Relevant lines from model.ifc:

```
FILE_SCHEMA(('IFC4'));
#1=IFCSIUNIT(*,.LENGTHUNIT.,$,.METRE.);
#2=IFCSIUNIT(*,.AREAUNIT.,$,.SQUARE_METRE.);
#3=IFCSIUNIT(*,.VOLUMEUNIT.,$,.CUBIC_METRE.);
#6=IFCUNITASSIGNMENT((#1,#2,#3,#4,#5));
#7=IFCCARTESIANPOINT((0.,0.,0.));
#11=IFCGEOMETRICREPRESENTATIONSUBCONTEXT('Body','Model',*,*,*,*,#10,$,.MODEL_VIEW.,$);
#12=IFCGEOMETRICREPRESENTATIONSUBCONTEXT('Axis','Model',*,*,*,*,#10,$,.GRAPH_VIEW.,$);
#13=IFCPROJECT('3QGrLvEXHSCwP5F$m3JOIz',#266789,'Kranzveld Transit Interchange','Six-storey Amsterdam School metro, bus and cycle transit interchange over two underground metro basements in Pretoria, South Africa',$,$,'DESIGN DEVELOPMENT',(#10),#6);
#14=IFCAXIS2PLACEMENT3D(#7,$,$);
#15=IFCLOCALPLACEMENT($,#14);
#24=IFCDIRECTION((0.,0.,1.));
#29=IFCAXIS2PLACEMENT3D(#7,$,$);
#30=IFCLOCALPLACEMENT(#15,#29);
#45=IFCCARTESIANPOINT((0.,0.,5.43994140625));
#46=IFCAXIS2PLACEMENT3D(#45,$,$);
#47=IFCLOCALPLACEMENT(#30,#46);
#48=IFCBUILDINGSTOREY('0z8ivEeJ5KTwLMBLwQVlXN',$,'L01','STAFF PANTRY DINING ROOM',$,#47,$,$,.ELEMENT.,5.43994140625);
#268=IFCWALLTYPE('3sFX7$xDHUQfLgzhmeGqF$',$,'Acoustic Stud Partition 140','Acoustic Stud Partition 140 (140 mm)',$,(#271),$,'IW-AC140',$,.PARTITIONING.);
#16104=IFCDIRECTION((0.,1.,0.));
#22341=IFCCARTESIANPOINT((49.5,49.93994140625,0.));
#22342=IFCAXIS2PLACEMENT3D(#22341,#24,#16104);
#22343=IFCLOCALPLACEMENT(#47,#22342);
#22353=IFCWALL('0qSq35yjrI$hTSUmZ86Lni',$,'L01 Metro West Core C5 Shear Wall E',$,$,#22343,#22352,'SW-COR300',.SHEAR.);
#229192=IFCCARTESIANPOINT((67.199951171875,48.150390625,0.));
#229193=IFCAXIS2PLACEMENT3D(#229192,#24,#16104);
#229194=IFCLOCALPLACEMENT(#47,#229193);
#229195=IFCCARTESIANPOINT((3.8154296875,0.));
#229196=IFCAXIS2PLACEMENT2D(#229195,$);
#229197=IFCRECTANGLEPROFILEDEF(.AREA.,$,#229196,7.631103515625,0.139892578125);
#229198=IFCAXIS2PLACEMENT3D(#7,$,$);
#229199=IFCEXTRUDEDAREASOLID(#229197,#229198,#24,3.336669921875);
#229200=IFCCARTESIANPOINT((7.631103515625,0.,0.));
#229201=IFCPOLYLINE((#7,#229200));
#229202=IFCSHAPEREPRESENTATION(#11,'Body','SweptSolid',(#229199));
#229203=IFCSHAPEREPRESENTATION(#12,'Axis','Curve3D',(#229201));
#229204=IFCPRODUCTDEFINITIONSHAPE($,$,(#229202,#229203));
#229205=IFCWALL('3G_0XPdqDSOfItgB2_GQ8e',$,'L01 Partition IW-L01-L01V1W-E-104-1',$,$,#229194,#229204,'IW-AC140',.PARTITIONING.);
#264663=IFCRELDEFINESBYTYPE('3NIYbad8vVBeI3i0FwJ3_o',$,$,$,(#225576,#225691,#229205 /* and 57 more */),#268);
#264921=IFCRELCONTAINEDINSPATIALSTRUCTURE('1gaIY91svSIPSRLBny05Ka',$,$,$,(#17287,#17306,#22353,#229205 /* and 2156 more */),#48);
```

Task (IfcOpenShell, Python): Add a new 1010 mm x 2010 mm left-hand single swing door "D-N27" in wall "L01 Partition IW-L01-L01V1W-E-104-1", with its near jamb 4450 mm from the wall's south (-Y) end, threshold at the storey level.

```python
import numpy as np
import ifcopenshell
import ifcopenshell.api.feature
import ifcopenshell.api.geometry
import ifcopenshell.api.root
import ifcopenshell.api.spatial
import ifcopenshell.geom
import ifcopenshell.util.element
import ifcopenshell.util.placement
import ifcopenshell.util.representation
import ifcopenshell.util.shape
import ifcopenshell.util.unit

model = ifcopenshell.open("model.ifc")
unit_scale = ifcopenshell.util.unit.calculate_unit_scale(model)
settings = ifcopenshell.geom.settings()


def volume(element):
    """Net volume in cubic metres, openings subtracted."""
    shape = ifcopenshell.geom.create_shape(settings, element)
    return ifcopenshell.util.shape.get_volume(shape.geometry)


wall = model.by_guid("3G_0XPdqDSOfItgB2_GQ8e")
storey = ifcopenshell.util.element.get_container(wall, ifc_class="IfcBuildingStorey")
context = ifcopenshell.util.representation.get_context(model, "Model", "Body", "MODEL_VIEW")
before = volume(wall)

width, height, from_end, sill = 1.01, 2.01, 4.45, 0.0  # metres

# The wall runs along its own X axis, and the end named is its -X end.
wall_shape = ifcopenshell.geom.create_shape(settings, wall)
x, y, z = ifcopenshell.util.shape.get_vertices(wall_shape.geometry).T
start = x.min() + from_end
face, thickness = float(y.min()), float(y.max() - y.min())
wall_matrix = ifcopenshell.util.placement.get_local_placement(wall.ObjectPlacement)
level = ifcopenshell.util.placement.get_local_placement(storey.ObjectPlacement)[2, 3]


def in_wall(x, y):
    """Placement at x, y metres in the wall's axes, at sill height."""
    matrix = wall_matrix.copy()
    matrix[:, 3] = wall_matrix @ np.array([x / unit_scale, y / unit_scale, 0.0, 1.0])
    matrix[2, 3] = level + sill / unit_scale
    return matrix


# Opening: a box that overshoots both wall faces by 50 mm.
opening = ifcopenshell.api.root.create_entity(model, ifc_class="IfcOpeningElement", predefined_type="OPENING")
box = ifcopenshell.api.geometry.add_wall_representation(
    model, context=context, length=width, height=height, thickness=thickness + 0.1
)
ifcopenshell.api.geometry.assign_representation(model, product=opening, representation=box)
ifcopenshell.api.geometry.edit_object_placement(model, product=opening, matrix=in_wall(start, face - 0.05), is_si=False)
ifcopenshell.api.feature.add_feature(model, feature=opening, element=wall)

door = ifcopenshell.api.root.create_entity(model, ifc_class="IfcDoor", name="D-N27", predefined_type="DOOR")
door.OverallWidth, door.OverallHeight = width / unit_scale, height / unit_scale
door.OperationType = "SINGLE_SWING_LEFT"
body = ifcopenshell.api.geometry.add_door_representation(
    model,
    context=context,
    overall_width=door.OverallWidth,
    overall_height=door.OverallHeight,
    operation_type="SINGLE_SWING_LEFT",
    lining_properties={"LiningDepth": thickness / unit_scale, "ThresholdDepth": thickness / unit_scale},
)
ifcopenshell.api.geometry.assign_representation(model, product=door, representation=body)
ifcopenshell.api.spatial.assign_container(model, products=[door], relating_structure=storey)
ifcopenshell.api.feature.add_filling(model, opening=opening, element=door)

# The lining spans the wall, so the door starts at the wall face.
ifcopenshell.api.geometry.edit_object_placement(model, product=door, matrix=in_wall(start, face), is_si=False)

after = volume(wall)

print(f"wall volume {before:.3f} -> {after:.3f} m3")

model.write("model-out.ifc")
```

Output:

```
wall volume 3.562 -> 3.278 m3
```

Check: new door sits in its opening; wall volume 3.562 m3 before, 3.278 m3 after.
